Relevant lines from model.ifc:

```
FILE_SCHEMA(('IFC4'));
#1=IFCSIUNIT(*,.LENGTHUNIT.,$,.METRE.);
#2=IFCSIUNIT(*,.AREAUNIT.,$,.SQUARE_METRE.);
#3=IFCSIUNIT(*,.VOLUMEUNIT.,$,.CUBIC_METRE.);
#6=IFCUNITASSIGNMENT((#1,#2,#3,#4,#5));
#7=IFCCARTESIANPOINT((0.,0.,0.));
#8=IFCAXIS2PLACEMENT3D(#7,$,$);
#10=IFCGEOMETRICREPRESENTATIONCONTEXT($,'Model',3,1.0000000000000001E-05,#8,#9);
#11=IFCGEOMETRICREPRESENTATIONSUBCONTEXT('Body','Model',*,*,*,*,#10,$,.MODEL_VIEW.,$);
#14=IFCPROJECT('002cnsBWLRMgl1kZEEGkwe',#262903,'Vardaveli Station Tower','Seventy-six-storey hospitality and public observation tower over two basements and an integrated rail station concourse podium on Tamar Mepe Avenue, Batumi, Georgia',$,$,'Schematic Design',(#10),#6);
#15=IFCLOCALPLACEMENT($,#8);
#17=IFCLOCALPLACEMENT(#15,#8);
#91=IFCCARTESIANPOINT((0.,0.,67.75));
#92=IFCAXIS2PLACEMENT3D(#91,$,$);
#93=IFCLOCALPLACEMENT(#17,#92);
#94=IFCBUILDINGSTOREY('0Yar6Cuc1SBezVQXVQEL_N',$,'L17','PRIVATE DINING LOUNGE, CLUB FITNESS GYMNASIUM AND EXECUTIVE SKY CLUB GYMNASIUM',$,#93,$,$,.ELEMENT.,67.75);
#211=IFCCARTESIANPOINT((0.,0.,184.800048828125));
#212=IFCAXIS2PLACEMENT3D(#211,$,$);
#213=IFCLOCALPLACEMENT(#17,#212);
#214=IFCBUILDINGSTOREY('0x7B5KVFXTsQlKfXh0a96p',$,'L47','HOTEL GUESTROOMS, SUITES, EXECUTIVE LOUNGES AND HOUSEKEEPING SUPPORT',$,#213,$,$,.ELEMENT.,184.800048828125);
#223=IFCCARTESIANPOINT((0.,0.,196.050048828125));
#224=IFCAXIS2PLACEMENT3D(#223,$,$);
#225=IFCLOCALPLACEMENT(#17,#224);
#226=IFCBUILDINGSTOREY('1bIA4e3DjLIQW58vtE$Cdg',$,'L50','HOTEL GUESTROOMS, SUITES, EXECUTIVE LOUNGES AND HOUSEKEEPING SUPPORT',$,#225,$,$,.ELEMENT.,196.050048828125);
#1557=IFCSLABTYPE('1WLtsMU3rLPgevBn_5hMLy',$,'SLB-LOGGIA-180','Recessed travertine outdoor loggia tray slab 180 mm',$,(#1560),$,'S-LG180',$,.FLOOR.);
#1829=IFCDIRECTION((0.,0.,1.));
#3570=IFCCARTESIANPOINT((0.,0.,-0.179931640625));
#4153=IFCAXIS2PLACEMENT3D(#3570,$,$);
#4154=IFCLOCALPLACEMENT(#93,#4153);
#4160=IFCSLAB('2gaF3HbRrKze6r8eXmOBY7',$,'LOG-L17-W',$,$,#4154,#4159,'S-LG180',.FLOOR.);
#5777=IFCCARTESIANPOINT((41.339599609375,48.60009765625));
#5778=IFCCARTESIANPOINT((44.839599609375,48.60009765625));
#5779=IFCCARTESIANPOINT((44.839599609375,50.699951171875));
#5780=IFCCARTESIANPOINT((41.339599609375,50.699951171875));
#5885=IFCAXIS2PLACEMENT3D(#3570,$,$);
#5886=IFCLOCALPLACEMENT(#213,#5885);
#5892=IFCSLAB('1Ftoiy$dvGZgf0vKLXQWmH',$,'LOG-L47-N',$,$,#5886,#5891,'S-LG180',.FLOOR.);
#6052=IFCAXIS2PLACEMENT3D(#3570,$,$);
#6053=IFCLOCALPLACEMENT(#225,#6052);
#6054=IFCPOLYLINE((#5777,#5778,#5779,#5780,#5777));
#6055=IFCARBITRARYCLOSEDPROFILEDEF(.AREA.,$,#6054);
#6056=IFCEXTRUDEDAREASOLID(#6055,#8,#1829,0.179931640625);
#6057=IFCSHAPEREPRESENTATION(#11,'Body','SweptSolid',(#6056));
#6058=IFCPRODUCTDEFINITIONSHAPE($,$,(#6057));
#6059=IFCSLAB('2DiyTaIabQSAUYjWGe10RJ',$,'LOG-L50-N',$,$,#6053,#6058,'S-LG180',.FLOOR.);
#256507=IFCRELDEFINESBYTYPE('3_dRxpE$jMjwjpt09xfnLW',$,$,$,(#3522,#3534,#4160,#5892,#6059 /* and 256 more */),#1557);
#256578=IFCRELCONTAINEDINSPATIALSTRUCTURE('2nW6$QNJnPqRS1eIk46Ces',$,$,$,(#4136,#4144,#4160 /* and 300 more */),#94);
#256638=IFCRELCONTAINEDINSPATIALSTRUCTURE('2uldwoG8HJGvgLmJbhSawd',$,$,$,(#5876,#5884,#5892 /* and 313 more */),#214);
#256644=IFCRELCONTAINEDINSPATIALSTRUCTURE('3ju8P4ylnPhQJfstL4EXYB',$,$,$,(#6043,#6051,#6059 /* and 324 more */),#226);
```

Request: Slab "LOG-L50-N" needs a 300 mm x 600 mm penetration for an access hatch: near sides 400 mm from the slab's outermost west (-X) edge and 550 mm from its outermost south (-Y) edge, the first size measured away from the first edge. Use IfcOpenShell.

```python
import numpy as np
import ifcopenshell
import ifcopenshell.api.feature
import ifcopenshell.api.geometry
import ifcopenshell.api.root
import ifcopenshell.geom
import ifcopenshell.util.placement
import ifcopenshell.util.representation
import ifcopenshell.util.shape
import ifcopenshell.util.unit

model = ifcopenshell.open("model.ifc")
unit_scale = ifcopenshell.util.unit.calculate_unit_scale(model)
settings = ifcopenshell.geom.settings()


def volume(element):
    """Net volume in cubic metres, openings subtracted."""
    shape = ifcopenshell.geom.create_shape(settings, element)
    return ifcopenshell.util.shape.get_volume(shape.geometry)


slab = model.by_guid("2DiyTaIabQSAUYjWGe10RJ")
before = volume(slab)

# Extent in the slab's own axes, in metres. The edges named are its -X and -Y sides.
slab_shape = ifcopenshell.geom.create_shape(settings, slab)
vertices = ifcopenshell.util.shape.get_vertices(slab_shape.geometry)
x_min, y_min, bottom = vertices.min(axis=0)
top = vertices[:, 2].max()

opening = ifcopenshell.api.root.create_entity(model, ifc_class="IfcOpeningElement", name="Access hatch opening", predefined_type="OPENING")
context = ifcopenshell.util.representation.get_context(model, "Model", "Body", "MODEL_VIEW")
width, depth = 0.3, 0.6
outline = [(0.0, 0.0), (width, 0.0), (width, depth), (0.0, depth), (0.0, 0.0)]
# Overshoot both faces by 50 mm so the cut is clean.
shape = ifcopenshell.api.geometry.add_slab_representation(
    model, context=context, depth=top - bottom + 0.1, polyline=outline
)
ifcopenshell.api.geometry.assign_representation(model, product=opening, representation=shape)

matrix = ifcopenshell.util.placement.get_local_placement(slab.ObjectPlacement)
matrix[:, 3] = matrix @ np.append(np.array([x_min + 0.4, y_min + 0.55, bottom - 0.05]) / unit_scale, 1.0)
ifcopenshell.api.geometry.edit_object_placement(model, product=opening, matrix=matrix, is_si=False)
ifcopenshell.api.feature.add_feature(model, feature=opening, element=slab)

after = volume(slab)

print(f"slab volume {before:.3f} -> {after:.3f} m3")

model.write("model_updated.ifc")
```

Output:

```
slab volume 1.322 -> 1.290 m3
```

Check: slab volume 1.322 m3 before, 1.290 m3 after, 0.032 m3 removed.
